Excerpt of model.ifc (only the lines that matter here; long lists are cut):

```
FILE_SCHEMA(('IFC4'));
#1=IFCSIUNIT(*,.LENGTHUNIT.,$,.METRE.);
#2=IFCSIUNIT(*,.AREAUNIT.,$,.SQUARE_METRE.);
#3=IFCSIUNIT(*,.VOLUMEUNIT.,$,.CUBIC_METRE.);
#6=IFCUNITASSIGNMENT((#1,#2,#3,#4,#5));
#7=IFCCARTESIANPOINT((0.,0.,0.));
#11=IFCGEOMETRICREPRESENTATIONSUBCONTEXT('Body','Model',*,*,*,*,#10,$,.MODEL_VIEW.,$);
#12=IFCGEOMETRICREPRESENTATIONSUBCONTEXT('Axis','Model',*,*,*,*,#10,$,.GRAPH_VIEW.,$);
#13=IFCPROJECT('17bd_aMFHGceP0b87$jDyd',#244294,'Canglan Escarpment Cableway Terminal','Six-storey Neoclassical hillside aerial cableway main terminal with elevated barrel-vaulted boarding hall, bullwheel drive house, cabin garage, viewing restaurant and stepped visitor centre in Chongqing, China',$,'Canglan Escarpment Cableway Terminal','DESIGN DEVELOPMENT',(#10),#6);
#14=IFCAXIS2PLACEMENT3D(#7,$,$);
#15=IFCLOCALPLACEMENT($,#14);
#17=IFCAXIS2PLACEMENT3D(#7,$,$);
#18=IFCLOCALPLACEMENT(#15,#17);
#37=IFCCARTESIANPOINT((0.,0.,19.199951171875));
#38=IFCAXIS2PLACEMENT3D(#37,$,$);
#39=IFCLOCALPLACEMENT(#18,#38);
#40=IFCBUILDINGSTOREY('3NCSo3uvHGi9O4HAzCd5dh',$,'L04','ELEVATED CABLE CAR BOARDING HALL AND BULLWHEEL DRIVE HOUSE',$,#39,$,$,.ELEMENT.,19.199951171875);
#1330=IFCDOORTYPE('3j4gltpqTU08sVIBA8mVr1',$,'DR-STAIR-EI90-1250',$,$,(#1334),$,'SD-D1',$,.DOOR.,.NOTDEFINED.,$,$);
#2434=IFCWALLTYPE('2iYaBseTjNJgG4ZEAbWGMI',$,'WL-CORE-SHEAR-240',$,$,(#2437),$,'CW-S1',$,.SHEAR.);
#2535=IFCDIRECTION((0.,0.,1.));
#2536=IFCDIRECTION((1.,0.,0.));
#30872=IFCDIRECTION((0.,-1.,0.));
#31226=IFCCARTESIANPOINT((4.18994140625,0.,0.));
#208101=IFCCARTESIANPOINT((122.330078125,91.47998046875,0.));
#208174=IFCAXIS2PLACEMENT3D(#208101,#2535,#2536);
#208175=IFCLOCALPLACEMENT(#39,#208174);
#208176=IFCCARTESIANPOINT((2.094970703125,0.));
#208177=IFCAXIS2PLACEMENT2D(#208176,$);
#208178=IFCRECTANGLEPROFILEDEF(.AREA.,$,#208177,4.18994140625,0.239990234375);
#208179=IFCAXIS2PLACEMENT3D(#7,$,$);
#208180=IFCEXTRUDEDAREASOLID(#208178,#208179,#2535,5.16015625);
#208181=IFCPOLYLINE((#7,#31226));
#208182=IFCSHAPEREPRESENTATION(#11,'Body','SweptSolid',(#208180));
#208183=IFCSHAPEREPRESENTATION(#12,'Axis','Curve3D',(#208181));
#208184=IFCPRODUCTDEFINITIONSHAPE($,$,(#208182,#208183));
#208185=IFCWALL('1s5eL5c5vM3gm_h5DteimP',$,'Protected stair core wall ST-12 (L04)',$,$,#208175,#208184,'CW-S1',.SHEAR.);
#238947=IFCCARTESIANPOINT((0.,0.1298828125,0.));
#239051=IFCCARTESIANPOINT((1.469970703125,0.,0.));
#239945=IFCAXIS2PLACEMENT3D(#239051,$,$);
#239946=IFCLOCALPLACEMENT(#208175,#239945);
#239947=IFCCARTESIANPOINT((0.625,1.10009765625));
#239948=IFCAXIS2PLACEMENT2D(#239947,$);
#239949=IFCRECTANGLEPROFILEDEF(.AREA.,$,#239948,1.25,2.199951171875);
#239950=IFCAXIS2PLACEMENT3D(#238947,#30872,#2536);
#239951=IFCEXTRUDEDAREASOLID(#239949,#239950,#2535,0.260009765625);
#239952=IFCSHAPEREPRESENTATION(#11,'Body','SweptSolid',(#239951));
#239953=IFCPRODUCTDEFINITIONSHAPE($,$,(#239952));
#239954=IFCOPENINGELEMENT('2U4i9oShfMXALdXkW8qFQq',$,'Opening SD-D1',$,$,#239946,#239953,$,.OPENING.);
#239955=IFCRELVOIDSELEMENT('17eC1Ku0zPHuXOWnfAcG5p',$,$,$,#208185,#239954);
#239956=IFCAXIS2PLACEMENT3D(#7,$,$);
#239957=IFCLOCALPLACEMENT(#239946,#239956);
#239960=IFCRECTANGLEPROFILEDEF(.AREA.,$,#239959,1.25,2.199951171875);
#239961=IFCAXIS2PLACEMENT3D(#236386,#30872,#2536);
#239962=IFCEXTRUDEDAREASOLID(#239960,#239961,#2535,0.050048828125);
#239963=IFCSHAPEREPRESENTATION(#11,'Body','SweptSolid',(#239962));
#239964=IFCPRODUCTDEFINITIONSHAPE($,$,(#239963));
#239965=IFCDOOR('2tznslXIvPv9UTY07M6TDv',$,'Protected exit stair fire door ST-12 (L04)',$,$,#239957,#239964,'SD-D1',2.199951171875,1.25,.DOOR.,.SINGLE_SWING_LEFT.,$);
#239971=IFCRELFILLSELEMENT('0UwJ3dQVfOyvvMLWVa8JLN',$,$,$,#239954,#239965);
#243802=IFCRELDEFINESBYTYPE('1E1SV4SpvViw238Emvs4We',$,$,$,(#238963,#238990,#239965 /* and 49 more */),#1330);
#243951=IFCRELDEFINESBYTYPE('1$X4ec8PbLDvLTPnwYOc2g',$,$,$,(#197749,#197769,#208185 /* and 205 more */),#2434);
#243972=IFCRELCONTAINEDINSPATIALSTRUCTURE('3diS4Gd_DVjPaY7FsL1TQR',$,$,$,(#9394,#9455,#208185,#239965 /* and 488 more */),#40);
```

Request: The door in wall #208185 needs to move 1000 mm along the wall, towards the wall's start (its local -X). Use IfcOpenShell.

```python
import ifcopenshell
import ifcopenshell.api.geometry
import ifcopenshell.util.placement
import ifcopenshell.util.unit

model = ifcopenshell.open("model.ifc")
unit_scale = ifcopenshell.util.unit.calculate_unit_scale(model)

door = model.by_guid("2tznslXIvPv9UTY07M6TDv")
opening = door.FillsVoids[0].RelatingOpeningElement
wall = opening.VoidsElements[0].RelatingBuildingElement

wall_matrix = ifcopenshell.util.placement.get_local_placement(wall.ObjectPlacement)
shift = wall_matrix[:3, 0] * -1 / unit_scale
before = ifcopenshell.util.placement.get_local_placement(door.ObjectPlacement)[:3, 3].copy()

# The door is placed relative to its opening, so it follows when the opening moves.
matrix = ifcopenshell.util.placement.get_local_placement(opening.ObjectPlacement)
matrix[:3, 3] += shift
ifcopenshell.api.geometry.edit_object_placement(
    model, product=opening, matrix=matrix, is_si=False, should_transform_children=True
)

after = ifcopenshell.util.placement.get_local_placement(door.ObjectPlacement)[:3, 3]
print("door moved by", (after - before).round(3) + 0.0)

model.write("model_edited.ifc")
```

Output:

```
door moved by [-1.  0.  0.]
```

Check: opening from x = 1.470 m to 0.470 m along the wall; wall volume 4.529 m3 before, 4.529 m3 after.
